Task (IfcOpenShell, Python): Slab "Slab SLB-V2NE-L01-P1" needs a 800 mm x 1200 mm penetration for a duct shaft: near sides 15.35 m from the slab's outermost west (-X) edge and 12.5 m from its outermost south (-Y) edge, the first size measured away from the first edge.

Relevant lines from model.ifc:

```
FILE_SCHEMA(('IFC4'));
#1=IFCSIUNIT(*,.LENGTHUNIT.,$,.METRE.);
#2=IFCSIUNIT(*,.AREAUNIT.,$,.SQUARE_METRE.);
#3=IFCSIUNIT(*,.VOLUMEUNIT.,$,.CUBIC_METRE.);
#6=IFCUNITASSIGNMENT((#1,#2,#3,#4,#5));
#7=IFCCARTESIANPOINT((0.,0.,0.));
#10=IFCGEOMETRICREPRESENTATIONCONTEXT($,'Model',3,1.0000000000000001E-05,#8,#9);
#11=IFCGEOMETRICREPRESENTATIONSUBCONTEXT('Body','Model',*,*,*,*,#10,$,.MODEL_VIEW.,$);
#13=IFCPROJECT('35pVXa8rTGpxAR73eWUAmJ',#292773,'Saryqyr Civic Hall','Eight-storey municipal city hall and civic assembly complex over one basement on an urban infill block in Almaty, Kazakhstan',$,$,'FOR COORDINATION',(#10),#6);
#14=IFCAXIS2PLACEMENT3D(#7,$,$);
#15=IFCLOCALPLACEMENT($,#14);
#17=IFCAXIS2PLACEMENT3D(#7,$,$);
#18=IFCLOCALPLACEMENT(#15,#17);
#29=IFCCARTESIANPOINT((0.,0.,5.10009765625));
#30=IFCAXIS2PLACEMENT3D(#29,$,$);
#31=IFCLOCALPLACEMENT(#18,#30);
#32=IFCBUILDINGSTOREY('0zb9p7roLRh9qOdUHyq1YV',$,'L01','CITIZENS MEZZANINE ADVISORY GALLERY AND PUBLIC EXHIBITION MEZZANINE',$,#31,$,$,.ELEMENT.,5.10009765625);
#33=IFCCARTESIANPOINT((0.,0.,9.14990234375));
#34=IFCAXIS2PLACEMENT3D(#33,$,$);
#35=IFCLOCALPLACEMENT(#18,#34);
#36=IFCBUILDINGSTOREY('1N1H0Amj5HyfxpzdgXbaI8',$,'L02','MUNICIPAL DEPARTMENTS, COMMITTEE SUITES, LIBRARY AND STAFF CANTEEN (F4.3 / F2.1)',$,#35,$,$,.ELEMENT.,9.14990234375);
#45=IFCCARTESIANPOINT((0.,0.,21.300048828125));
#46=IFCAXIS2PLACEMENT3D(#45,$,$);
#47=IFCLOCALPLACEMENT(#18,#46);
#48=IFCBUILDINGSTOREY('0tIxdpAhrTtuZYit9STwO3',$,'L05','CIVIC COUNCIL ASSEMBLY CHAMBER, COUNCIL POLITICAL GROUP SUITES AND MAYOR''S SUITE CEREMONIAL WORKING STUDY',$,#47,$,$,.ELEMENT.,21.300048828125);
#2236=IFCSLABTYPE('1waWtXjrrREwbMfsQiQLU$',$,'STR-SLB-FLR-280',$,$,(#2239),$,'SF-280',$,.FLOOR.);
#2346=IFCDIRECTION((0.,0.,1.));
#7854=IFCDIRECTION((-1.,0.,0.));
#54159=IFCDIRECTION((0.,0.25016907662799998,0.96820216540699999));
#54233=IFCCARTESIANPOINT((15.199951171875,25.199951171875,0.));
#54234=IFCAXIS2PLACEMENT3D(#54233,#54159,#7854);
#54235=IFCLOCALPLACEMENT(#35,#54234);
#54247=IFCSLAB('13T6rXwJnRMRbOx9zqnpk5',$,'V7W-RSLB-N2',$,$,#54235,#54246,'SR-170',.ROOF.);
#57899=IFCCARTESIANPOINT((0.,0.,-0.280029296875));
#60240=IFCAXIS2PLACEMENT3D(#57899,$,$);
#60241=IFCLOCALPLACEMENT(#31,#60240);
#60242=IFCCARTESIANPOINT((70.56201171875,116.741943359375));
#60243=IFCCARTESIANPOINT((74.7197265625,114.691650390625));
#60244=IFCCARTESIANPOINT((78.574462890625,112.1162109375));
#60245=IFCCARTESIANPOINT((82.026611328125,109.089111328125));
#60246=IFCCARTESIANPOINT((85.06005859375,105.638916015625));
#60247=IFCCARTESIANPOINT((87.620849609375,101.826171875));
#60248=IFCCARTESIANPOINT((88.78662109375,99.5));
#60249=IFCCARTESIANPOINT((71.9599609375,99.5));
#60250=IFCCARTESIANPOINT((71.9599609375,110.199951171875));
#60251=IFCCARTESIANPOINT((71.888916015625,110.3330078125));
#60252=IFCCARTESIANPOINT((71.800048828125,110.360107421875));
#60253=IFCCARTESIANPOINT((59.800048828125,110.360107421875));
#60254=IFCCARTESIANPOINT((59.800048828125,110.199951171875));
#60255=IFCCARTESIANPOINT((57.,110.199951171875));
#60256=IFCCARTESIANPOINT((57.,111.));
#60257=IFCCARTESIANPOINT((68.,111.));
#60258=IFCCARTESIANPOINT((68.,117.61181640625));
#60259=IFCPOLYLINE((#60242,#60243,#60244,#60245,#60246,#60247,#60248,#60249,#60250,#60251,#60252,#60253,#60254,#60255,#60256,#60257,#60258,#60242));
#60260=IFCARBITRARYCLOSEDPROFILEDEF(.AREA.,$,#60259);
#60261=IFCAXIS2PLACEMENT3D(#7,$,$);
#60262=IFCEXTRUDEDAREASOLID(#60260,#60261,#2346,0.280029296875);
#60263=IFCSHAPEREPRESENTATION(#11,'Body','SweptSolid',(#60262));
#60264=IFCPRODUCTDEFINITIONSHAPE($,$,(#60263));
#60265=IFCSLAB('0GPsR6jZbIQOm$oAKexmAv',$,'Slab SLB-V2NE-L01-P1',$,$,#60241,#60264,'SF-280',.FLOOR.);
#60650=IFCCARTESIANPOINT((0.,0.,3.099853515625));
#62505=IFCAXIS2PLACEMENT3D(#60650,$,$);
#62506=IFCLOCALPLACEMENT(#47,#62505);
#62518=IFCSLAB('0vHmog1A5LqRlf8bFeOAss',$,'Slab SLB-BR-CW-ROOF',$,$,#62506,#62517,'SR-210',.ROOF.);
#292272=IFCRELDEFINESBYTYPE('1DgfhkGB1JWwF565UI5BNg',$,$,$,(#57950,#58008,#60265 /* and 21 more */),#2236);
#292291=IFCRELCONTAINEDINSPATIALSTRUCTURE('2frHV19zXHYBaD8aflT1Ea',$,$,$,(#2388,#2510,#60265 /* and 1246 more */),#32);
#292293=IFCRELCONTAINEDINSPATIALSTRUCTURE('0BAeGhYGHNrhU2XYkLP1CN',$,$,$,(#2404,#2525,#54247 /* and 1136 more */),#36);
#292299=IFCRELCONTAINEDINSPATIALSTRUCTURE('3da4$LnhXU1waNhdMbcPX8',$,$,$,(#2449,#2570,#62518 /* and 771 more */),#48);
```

```python
import numpy as np
import ifcopenshell
import ifcopenshell.api.feature
import ifcopenshell.api.geometry
import ifcopenshell.api.root
import ifcopenshell.geom
import ifcopenshell.util.placement
import ifcopenshell.util.representation
import ifcopenshell.util.shape
import ifcopenshell.util.unit

model = ifcopenshell.open("model.ifc")
unit_scale = ifcopenshell.util.unit.calculate_unit_scale(model)
settings = ifcopenshell.geom.settings()


def volume(element):
    """Net volume in cubic metres, openings subtracted."""
    shape = ifcopenshell.geom.create_shape(settings, element)
    return ifcopenshell.util.shape.get_volume(shape.geometry)


slab = model.by_guid("0GPsR6jZbIQOm$oAKexmAv")
before = volume(slab)

# Extent in the slab's own axes, in metres. The edges named are its -X and -Y sides.
slab_shape = ifcopenshell.geom.create_shape(settings, slab)
vertices = ifcopenshell.util.shape.get_vertices(slab_shape.geometry)
x_min, y_min, bottom = vertices.min(axis=0)
top = vertices[:, 2].max()

opening = ifcopenshell.api.root.create_entity(model, ifc_class="IfcOpeningElement", name="Duct shaft opening", predefined_type="OPENING")
context = ifcopenshell.util.representation.get_context(model, "Model", "Body", "MODEL_VIEW")
width, depth = 0.8, 1.2
outline = [(0.0, 0.0), (width, 0.0), (width, depth), (0.0, depth), (0.0, 0.0)]
# Overshoot both faces by 50 mm so the cut is clean.
shape = ifcopenshell.api.geometry.add_slab_representation(
    model, context=context, depth=top - bottom + 0.1, polyline=outline
)
ifcopenshell.api.geometry.assign_representation(model, product=opening, representation=shape)

matrix = ifcopenshell.util.placement.get_local_placement(slab.ObjectPlacement)
matrix[:, 3] = matrix @ np.append(np.array([x_min + 15.35, y_min + 12.5, bottom - 0.05]) / unit_scale, 1.0)
ifcopenshell.api.geometry.edit_object_placement(model, product=opening, matrix=matrix, is_si=False)
ifcopenshell.api.feature.add_feature(model, feature=opening, element=slab)

after = volume(slab)

print(f"slab volume {before:.3f} -> {after:.3f} m3")

model.write("model_edited.ifc")
```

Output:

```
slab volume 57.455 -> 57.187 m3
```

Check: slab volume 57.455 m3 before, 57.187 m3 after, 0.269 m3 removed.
